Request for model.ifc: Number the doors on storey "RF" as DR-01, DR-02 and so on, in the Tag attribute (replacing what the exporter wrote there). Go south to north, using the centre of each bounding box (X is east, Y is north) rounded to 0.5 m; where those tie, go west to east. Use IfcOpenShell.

First a look at what the model holds.

```python
import ifcopenshell
import ifcopenshell.util.element
import ifcopenshell.util.placement

model = ifcopenshell.open("model.ifc")
print(model.schema)
storey = next(s for s in model.by_type("IfcBuildingStorey") if s.Name == "RF")
doors = [e for e in ifcopenshell.util.element.get_decomposition(storey) if e.is_a("IfcDoor")]
for e in sorted(doors, key=lambda e: e.id()):
    origin = ifcopenshell.util.placement.get_local_placement(e.ObjectPlacement)[:3, 3]
    print(e.id(), e.Tag, e.Name, origin.round(2) + 0.0, sep=" | ")
```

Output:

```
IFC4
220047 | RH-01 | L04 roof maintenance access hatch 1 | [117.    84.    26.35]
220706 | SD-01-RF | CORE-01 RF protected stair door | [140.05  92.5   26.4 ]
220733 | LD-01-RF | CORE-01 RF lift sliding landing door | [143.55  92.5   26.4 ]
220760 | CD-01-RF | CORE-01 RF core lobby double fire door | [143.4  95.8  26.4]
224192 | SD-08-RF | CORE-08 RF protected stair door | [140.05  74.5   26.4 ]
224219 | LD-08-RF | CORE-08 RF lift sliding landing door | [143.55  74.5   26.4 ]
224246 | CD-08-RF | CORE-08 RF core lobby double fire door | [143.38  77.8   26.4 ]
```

```python
import ifcopenshell
import ifcopenshell.geom
import ifcopenshell.util.element
import ifcopenshell.util.shape

model = ifcopenshell.open("model.ifc")
settings = ifcopenshell.geom.settings()
settings.set("use-world-coords", True)


def centre(element):
    shape = ifcopenshell.geom.create_shape(settings, element)
    return ifcopenshell.util.shape.get_bbox_centroid(shape.geometry)


storey = next(s for s in model.by_type("IfcBuildingStorey") if s.Name == "RF")
doors = [e for e in ifcopenshell.util.element.get_decomposition(storey) if e.is_a("IfcDoor")]

# Insertion points can sit at a corner or the storey origin, so sort by the geometry (in metres).
centres = {e: centre(e) for e in doors}
doors.sort(key=lambda e: (round(centres[e][1] / 0.5), centres[e][0]))

for i, e in enumerate(doors, start=1):
    number = f"DR-{i:02d}"
    e.Tag = number
    print(e.id(), number)

model.write("model-out.ifc")
```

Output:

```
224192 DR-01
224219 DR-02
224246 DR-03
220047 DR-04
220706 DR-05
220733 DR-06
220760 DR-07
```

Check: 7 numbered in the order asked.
